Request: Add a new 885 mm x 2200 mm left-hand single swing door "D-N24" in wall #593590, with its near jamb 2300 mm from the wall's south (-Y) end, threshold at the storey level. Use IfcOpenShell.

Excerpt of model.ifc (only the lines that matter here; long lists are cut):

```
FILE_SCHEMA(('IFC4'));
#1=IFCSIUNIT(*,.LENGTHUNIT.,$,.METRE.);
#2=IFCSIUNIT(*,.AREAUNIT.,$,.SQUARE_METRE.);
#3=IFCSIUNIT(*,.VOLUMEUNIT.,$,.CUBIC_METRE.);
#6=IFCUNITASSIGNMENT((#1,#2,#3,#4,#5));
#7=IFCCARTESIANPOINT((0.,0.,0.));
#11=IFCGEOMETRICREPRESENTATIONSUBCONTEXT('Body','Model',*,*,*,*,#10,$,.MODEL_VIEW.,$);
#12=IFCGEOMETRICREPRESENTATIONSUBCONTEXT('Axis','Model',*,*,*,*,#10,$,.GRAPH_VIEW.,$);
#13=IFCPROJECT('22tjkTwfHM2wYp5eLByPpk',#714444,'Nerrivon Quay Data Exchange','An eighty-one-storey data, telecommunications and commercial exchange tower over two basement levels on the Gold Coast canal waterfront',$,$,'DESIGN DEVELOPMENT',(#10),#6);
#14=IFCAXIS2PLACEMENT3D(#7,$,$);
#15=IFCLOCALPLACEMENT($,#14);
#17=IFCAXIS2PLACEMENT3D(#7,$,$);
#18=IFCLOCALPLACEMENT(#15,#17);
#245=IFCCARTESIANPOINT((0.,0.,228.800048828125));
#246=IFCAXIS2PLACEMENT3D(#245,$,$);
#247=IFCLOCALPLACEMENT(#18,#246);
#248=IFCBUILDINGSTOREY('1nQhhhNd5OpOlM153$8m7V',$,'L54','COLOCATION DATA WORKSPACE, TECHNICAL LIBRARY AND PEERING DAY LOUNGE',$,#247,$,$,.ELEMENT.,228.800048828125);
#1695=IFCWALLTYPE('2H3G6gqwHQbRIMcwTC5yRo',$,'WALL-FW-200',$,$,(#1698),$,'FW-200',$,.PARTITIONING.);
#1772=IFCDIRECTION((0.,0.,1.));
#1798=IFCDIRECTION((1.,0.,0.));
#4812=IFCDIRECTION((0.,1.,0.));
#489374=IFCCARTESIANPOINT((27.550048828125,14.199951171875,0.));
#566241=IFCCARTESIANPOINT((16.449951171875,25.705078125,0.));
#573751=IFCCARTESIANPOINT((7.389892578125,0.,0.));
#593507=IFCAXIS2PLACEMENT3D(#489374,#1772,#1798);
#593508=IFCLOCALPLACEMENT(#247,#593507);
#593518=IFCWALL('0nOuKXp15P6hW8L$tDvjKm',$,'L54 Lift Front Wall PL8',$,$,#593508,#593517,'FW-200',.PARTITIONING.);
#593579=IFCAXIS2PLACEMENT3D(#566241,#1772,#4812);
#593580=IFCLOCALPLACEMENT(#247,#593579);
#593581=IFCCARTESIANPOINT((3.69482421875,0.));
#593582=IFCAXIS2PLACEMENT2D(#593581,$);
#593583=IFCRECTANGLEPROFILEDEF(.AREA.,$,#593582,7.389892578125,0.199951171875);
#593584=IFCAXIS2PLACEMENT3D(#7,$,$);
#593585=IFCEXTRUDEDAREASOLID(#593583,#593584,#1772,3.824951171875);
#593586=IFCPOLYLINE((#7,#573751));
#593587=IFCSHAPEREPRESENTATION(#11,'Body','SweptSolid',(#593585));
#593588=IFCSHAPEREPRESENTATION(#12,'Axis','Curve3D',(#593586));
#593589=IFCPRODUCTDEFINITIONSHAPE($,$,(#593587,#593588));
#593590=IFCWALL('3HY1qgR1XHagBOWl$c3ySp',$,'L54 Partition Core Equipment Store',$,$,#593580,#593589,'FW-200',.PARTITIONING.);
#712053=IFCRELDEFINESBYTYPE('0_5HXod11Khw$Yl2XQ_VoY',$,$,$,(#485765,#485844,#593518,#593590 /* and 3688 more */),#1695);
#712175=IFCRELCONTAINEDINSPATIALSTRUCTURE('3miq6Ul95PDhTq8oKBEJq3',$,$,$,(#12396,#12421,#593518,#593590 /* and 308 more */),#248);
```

```python
import numpy as np
import ifcopenshell
import ifcopenshell.api.feature
import ifcopenshell.api.geometry
import ifcopenshell.api.root
import ifcopenshell.api.spatial
import ifcopenshell.geom
import ifcopenshell.util.element
import ifcopenshell.util.placement
import ifcopenshell.util.representation
import ifcopenshell.util.shape
import ifcopenshell.util.unit

model = ifcopenshell.open("model.ifc")
unit_scale = ifcopenshell.util.unit.calculate_unit_scale(model)
settings = ifcopenshell.geom.settings()


def volume(element):
    """Net volume in cubic metres, openings subtracted."""
    shape = ifcopenshell.geom.create_shape(settings, element)
    return ifcopenshell.util.shape.get_volume(shape.geometry)


wall = model.by_guid("3HY1qgR1XHagBOWl$c3ySp")
storey = ifcopenshell.util.element.get_container(wall, ifc_class="IfcBuildingStorey")
context = ifcopenshell.util.representation.get_context(model, "Model", "Body", "MODEL_VIEW")
before = volume(wall)

width, height, from_end, sill = 0.885, 2.2, 2.3, 0.0  # metres

# The wall runs along its own X axis, and the end named is its -X end.
wall_shape = ifcopenshell.geom.create_shape(settings, wall)
x, y, z = ifcopenshell.util.shape.get_vertices(wall_shape.geometry).T
start = x.min() + from_end
face, thickness = float(y.min()), float(y.max() - y.min())
wall_matrix = ifcopenshell.util.placement.get_local_placement(wall.ObjectPlacement)
level = ifcopenshell.util.placement.get_local_placement(storey.ObjectPlacement)[2, 3]


def in_wall(x, y):
    """Placement at x, y metres in the wall's axes, at sill height."""
    matrix = wall_matrix.copy()
    matrix[:, 3] = wall_matrix @ np.array([x / unit_scale, y / unit_scale, 0.0, 1.0])
    matrix[2, 3] = level + sill / unit_scale
    return matrix


# Opening: a box that overshoots both wall faces by 50 mm.
opening = ifcopenshell.api.root.create_entity(model, ifc_class="IfcOpeningElement", predefined_type="OPENING")
box = ifcopenshell.api.geometry.add_wall_representation(
    model, context=context, length=width, height=height, thickness=thickness + 0.1
)
ifcopenshell.api.geometry.assign_representation(model, product=opening, representation=box)
ifcopenshell.api.geometry.edit_object_placement(model, product=opening, matrix=in_wall(start, face - 0.05), is_si=False)
ifcopenshell.api.feature.add_feature(model, feature=opening, element=wall)

door = ifcopenshell.api.root.create_entity(model, ifc_class="IfcDoor", name="D-N24", predefined_type="DOOR")
door.OverallWidth, door.OverallHeight = width / unit_scale, height / unit_scale
door.OperationType = "SINGLE_SWING_LEFT"
body = ifcopenshell.api.geometry.add_door_representation(
    model,
    context=context,
    overall_width=door.OverallWidth,
    overall_height=door.OverallHeight,
    operation_type="SINGLE_SWING_LEFT",
    lining_properties={"LiningDepth": thickness / unit_scale, "ThresholdDepth": thickness / unit_scale},
)
ifcopenshell.api.geometry.assign_representation(model, product=door, representation=body)
ifcopenshell.api.spatial.assign_container(model, products=[door], relating_structure=storey)
ifcopenshell.api.feature.add_filling(model, opening=opening, element=door)

# The lining spans the wall, so the door starts at the wall face.
ifcopenshell.api.geometry.edit_object_placement(model, product=door, matrix=in_wall(start, face), is_si=False)

after = volume(wall)

print(f"wall volume {before:.3f} -> {after:.3f} m3")

model.write("model_rev.ifc")
```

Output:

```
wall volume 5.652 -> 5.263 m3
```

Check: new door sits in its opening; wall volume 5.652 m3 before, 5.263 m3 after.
